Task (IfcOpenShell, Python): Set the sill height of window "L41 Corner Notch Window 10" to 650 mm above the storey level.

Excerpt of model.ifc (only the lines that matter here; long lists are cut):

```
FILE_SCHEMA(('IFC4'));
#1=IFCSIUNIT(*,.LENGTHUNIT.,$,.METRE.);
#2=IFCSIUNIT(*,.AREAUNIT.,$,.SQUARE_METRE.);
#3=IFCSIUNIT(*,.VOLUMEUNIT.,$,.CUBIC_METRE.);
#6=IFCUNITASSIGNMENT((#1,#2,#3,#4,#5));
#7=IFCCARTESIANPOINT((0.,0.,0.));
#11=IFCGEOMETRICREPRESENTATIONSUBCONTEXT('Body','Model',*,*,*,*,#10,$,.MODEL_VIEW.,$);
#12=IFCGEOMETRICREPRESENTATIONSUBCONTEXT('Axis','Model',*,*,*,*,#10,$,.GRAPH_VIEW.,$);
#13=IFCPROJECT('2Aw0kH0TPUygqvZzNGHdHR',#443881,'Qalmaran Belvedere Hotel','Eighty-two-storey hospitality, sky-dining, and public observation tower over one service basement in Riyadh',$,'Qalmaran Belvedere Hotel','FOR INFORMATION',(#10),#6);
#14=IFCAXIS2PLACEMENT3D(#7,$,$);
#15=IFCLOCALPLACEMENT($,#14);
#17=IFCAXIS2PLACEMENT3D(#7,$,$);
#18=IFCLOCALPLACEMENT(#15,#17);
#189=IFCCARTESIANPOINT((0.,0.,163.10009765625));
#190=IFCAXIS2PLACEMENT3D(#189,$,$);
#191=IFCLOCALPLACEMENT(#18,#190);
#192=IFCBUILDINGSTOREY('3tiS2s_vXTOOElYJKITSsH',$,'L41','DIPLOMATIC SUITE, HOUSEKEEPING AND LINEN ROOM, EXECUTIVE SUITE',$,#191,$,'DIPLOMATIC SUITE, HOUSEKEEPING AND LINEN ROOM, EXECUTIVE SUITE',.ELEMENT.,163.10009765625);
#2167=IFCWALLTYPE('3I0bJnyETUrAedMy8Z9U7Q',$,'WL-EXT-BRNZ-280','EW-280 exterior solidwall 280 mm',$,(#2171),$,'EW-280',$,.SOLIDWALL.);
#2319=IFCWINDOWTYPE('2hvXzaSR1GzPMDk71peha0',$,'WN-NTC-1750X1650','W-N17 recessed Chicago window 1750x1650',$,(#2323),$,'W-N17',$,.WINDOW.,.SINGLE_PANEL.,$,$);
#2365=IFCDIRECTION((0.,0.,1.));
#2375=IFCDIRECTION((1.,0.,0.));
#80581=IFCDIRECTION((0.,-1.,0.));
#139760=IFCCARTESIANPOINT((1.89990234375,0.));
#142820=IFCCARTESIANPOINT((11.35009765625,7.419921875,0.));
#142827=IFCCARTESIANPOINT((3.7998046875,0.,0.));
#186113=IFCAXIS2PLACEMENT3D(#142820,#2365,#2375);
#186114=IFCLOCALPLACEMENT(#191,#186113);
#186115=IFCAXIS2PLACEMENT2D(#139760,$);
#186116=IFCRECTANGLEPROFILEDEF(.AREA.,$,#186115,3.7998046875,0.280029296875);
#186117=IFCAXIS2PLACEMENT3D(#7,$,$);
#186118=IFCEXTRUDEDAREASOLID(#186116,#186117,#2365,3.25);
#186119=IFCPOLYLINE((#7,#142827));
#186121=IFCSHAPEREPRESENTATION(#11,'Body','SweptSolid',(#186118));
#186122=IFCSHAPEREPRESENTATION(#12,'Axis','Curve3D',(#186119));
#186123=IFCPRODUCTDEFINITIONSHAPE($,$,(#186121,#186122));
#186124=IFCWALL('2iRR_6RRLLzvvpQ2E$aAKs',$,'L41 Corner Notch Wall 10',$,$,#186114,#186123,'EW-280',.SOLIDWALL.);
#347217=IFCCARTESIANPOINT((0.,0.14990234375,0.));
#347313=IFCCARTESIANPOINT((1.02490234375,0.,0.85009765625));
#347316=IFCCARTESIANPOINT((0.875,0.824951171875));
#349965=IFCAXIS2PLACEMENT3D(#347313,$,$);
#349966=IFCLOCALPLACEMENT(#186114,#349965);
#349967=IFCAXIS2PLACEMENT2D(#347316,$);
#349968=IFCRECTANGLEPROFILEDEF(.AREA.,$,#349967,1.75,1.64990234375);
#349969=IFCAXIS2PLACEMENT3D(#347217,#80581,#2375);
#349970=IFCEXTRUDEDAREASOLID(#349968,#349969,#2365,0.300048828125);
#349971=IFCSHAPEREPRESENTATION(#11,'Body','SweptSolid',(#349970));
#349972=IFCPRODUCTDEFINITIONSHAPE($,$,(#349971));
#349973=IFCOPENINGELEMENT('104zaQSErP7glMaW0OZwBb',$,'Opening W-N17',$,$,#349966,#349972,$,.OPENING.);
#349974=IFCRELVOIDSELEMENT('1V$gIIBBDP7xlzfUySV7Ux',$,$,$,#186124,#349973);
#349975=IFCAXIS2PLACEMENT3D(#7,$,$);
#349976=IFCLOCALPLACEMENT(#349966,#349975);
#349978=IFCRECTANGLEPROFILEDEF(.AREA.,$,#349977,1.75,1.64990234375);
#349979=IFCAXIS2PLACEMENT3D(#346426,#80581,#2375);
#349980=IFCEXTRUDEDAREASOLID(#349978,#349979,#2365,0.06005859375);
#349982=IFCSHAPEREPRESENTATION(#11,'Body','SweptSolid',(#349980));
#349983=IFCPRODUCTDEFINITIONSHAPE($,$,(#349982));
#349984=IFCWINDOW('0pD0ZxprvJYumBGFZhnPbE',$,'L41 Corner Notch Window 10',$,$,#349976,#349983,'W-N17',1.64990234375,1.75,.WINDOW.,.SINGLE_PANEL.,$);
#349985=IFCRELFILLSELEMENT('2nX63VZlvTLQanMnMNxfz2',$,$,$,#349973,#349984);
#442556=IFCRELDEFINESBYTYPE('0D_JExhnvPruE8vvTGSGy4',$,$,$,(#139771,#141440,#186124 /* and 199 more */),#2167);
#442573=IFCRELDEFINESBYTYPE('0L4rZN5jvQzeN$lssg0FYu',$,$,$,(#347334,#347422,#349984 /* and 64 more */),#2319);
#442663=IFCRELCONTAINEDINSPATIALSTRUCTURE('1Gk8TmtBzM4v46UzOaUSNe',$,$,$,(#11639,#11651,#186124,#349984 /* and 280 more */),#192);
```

```python
import numpy as np
import ifcopenshell
import ifcopenshell.api.geometry
import ifcopenshell.geom
import ifcopenshell.util.element
import ifcopenshell.util.placement
import ifcopenshell.util.shape
import ifcopenshell.util.unit

model = ifcopenshell.open("model.ifc")
unit_scale = ifcopenshell.util.unit.calculate_unit_scale(model)

window = model.by_guid("0pD0ZxprvJYumBGFZhnPbE")
opening = window.FillsVoids[0].RelatingOpeningElement
storey = ifcopenshell.util.element.get_container(window, ifc_class="IfcBuildingStorey")
level = ifcopenshell.util.placement.get_local_placement(storey.ObjectPlacement)[2, 3]

# The opening's origin need not be at the sill, so measure its lowest point.
shape = ifcopenshell.geom.create_shape(ifcopenshell.geom.settings(), opening)
bottom = ifcopenshell.util.shape.get_shape_bottom_elevation(shape, shape.geometry) / unit_scale
dz = level + 0.65 / unit_scale - bottom

shift = np.array([0.0, 0.0, dz])
# The window is placed relative to its opening, so it follows when the opening moves.
matrix = ifcopenshell.util.placement.get_local_placement(opening.ObjectPlacement)
matrix[:3, 3] += shift
ifcopenshell.api.geometry.edit_object_placement(
    model, product=opening, matrix=matrix, is_si=False, should_transform_children=True
)

print(f"moved by {dz * unit_scale:+.3f} m")

model.write("model_edited.ifc")
```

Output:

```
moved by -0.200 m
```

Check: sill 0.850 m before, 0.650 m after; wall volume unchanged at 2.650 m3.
